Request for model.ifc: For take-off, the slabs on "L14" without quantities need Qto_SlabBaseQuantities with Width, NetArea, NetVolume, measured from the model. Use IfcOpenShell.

First a look at what the model holds.

```python
import ifcopenshell
import ifcopenshell.util.element
import ifcopenshell.util.unit

model = ifcopenshell.open("model.ifc")
print(model.schema)
for unit_type in ("LENGTHUNIT", "AREAUNIT", "VOLUMEUNIT"):
    print(unit_type, ifcopenshell.util.unit.calculate_unit_scale(model, unit_type))
storey = next(s for s in model.by_type("IfcBuildingStorey") if s.Name == "L14")
slabs = [e for e in ifcopenshell.util.element.get_decomposition(storey) if e.is_a("IfcSlab")]
for e in sorted(slabs, key=lambda e: e.id()):
    print(e.id(), e.is_a(), e.Name, list(ifcopenshell.util.element.get_psets(e, qtos_only=True)), sep=" | ")
```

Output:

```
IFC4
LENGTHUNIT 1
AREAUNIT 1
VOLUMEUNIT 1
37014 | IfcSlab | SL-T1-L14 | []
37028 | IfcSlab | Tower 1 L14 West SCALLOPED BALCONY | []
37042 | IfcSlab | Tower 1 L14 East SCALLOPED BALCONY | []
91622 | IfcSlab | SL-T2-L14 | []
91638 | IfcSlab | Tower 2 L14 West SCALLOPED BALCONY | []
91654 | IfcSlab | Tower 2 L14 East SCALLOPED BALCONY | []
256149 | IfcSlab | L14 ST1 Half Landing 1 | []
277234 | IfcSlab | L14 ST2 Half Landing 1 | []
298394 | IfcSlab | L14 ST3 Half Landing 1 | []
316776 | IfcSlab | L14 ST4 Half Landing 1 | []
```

```python
import ifcopenshell
import ifcopenshell.api.pset
import ifcopenshell.geom
import ifcopenshell.util.element
import ifcopenshell.util.shape
import ifcopenshell.util.unit

model = ifcopenshell.open("model.ifc")
unit_scale = ifcopenshell.util.unit.calculate_unit_scale(model)
area_scale = ifcopenshell.util.unit.calculate_unit_scale(model, "AREAUNIT")
volume_scale = ifcopenshell.util.unit.calculate_unit_scale(model, "VOLUMEUNIT")
settings = ifcopenshell.geom.settings()

storey = next(s for s in model.by_type("IfcBuildingStorey") if s.Name == "L14")
slabs = [e for e in ifcopenshell.util.element.get_decomposition(storey) if e.is_a("IfcSlab")]

for e in sorted(slabs, key=lambda e: e.id()):
    if ifcopenshell.util.element.get_psets(e, qtos_only=True, should_inherit=False):
        continue
    # Geometry comes back in metres, in the element's own axes.
    shape = ifcopenshell.geom.create_shape(settings, e)
    values = {
        "Width": ifcopenshell.util.shape.get_z(shape.geometry) / unit_scale,
        "NetArea": ifcopenshell.util.shape.get_footprint_area(shape.geometry) / area_scale,
        "NetVolume": ifcopenshell.util.shape.get_volume(shape.geometry) / volume_scale,
    }
    qto = ifcopenshell.api.pset.add_qto(model, product=e, name="Qto_SlabBaseQuantities")
    ifcopenshell.api.pset.edit_qto(model, qto=qto, properties=values)
    print(e.id(), {k: round(v, 3) for k, v in values.items()})

model.write("model_rev.ifc")
```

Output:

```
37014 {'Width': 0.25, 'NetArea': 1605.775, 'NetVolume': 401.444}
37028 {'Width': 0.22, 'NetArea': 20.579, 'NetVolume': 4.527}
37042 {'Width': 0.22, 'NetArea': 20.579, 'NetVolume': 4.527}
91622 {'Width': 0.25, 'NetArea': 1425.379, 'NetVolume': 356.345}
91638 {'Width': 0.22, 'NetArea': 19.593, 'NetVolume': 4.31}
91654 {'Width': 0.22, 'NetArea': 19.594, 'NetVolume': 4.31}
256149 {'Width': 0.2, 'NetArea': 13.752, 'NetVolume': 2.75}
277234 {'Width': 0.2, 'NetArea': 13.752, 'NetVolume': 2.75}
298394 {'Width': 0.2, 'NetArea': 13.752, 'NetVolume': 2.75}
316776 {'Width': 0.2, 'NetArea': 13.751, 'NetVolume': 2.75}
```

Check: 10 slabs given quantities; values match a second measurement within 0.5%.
